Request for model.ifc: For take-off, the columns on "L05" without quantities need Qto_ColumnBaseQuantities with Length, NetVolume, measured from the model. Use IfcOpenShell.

First a look at what the model holds.

```python
import ifcopenshell
import ifcopenshell.util.element
import ifcopenshell.util.unit

model = ifcopenshell.open("model.ifc")
print(model.schema)
for unit_type in ("LENGTHUNIT", "AREAUNIT", "VOLUMEUNIT"):
    print(unit_type, ifcopenshell.util.unit.calculate_unit_scale(model, unit_type))
storey = next(s for s in model.by_type("IfcBuildingStorey") if s.Name == "L05")
columns = [e for e in ifcopenshell.util.element.get_decomposition(storey) if e.is_a("IfcColumn")]
for e in sorted(columns, key=lambda e: e.id()):
    print(e.id(), e.is_a(), e.Name, list(ifcopenshell.util.element.get_psets(e, qtos_only=True)), sep=" | ")
```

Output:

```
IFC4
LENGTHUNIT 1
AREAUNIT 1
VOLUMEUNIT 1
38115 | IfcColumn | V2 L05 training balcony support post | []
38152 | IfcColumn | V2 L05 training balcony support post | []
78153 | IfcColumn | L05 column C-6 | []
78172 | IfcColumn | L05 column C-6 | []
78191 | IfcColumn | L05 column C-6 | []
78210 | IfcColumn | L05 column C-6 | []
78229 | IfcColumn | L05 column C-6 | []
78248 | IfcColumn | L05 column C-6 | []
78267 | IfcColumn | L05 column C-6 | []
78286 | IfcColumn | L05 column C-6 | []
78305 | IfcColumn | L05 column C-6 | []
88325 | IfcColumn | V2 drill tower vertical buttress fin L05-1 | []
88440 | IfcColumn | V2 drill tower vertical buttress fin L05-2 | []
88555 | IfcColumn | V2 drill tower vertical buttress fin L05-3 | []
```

```python
import ifcopenshell
import ifcopenshell.api.pset
import ifcopenshell.geom
import ifcopenshell.util.element
import ifcopenshell.util.shape
import ifcopenshell.util.unit

model = ifcopenshell.open("model.ifc")
unit_scale = ifcopenshell.util.unit.calculate_unit_scale(model)
volume_scale = ifcopenshell.util.unit.calculate_unit_scale(model, "VOLUMEUNIT")
settings = ifcopenshell.geom.settings()

storey = next(s for s in model.by_type("IfcBuildingStorey") if s.Name == "L05")
columns = [e for e in ifcopenshell.util.element.get_decomposition(storey) if e.is_a("IfcColumn")]

for e in sorted(columns, key=lambda e: e.id()):
    if ifcopenshell.util.element.get_psets(e, qtos_only=True, should_inherit=False):
        continue
    # Geometry comes back in metres, in the element's own axes.
    shape = ifcopenshell.geom.create_shape(settings, e)
    values = {
        "Length": ifcopenshell.util.shape.get_z(shape.geometry) / unit_scale,
        "NetVolume": ifcopenshell.util.shape.get_volume(shape.geometry) / volume_scale,
    }
    qto = ifcopenshell.api.pset.add_qto(model, product=e, name="Qto_ColumnBaseQuantities")
    ifcopenshell.api.pset.edit_qto(model, qto=qto, properties=values)
    print(e.id(), {k: round(v, 3) for k, v in values.items()})

model.write("model_v2.ifc")
```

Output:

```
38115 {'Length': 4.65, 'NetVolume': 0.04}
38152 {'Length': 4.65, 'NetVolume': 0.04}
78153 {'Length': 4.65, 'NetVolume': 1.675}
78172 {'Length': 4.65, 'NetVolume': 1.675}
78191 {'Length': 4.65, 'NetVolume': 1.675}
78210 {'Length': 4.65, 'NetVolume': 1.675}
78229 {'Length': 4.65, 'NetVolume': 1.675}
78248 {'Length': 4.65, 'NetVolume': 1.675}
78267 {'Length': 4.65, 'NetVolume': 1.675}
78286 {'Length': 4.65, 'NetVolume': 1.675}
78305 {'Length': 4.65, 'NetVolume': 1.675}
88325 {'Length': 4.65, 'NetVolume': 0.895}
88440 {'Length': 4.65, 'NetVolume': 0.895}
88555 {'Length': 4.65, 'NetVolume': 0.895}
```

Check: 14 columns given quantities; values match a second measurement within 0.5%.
